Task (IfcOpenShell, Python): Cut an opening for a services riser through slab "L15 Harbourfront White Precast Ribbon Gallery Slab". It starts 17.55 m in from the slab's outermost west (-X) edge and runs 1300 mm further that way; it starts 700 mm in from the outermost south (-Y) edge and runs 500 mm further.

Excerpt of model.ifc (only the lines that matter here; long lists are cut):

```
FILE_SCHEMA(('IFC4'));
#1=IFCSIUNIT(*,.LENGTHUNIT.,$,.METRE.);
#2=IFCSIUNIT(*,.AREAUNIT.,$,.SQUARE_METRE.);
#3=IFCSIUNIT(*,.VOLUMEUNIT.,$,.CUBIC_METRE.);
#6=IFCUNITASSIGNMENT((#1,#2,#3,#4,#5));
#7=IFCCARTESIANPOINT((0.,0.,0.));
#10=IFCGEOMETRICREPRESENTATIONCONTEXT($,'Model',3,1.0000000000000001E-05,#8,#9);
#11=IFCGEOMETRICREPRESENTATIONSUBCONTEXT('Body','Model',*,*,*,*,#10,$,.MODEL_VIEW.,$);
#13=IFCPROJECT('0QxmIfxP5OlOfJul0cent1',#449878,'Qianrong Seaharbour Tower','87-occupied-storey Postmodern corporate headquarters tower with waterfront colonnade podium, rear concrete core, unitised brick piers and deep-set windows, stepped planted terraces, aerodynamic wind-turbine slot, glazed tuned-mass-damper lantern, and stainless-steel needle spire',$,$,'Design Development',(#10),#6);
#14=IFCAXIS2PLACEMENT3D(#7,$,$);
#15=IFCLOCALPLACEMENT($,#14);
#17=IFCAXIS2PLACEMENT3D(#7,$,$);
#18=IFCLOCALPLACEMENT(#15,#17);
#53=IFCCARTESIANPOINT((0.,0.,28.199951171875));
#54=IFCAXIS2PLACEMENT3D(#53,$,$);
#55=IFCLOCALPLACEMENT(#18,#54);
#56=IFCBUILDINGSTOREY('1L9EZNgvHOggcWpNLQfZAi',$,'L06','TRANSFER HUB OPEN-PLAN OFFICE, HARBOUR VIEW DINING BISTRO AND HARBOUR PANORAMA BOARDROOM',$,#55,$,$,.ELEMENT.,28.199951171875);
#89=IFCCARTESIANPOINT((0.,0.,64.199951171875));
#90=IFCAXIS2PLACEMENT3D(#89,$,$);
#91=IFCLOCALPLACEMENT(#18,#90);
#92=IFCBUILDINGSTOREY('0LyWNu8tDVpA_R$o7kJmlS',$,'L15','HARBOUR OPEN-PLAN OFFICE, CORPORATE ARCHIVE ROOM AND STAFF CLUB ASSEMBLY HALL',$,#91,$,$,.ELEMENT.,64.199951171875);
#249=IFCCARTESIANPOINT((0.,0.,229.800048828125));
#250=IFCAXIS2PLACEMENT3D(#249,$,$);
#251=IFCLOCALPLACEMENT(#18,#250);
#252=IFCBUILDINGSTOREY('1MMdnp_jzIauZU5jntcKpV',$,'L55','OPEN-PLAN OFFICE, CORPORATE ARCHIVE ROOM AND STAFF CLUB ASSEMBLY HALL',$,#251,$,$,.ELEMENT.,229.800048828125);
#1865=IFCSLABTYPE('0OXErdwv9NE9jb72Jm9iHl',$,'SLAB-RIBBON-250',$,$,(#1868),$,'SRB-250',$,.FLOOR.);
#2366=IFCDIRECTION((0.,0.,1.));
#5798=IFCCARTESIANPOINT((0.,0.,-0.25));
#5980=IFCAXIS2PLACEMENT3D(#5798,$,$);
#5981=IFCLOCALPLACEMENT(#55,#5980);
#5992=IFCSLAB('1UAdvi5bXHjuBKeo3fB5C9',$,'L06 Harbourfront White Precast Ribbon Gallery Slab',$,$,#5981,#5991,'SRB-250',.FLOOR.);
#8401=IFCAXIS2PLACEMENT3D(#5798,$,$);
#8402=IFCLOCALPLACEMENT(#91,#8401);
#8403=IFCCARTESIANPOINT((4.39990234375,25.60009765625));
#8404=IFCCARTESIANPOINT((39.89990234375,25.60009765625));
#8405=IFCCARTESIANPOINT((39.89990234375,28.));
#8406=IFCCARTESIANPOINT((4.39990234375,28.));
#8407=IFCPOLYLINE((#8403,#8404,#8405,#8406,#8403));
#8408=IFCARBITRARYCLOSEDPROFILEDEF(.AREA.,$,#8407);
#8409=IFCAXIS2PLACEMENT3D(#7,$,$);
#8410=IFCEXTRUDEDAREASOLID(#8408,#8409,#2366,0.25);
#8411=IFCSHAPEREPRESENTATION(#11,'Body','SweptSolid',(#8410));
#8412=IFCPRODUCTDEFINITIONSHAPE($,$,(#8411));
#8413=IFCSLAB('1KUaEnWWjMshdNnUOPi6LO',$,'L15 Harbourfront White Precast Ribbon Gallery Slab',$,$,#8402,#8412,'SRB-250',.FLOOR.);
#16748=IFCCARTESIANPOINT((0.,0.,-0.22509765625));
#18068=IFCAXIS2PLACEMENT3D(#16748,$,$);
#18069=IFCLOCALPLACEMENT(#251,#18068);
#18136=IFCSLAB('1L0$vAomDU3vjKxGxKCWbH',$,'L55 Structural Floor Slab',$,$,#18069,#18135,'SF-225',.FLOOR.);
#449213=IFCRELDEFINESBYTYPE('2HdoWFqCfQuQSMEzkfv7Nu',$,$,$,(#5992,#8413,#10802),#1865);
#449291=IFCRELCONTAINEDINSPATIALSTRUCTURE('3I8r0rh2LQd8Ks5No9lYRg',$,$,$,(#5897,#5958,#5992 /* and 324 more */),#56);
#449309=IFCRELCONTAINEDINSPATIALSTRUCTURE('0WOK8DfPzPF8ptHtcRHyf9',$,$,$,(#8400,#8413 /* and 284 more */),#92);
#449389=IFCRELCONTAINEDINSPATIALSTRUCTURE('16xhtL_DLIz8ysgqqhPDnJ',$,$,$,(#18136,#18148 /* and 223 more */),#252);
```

```python
import numpy as np
import ifcopenshell
import ifcopenshell.api.feature
import ifcopenshell.api.geometry
import ifcopenshell.api.root
import ifcopenshell.geom
import ifcopenshell.util.placement
import ifcopenshell.util.representation
import ifcopenshell.util.shape
import ifcopenshell.util.unit

model = ifcopenshell.open("model.ifc")
unit_scale = ifcopenshell.util.unit.calculate_unit_scale(model)
settings = ifcopenshell.geom.settings()


def volume(element):
    """Net volume in cubic metres, openings subtracted."""
    shape = ifcopenshell.geom.create_shape(settings, element)
    return ifcopenshell.util.shape.get_volume(shape.geometry)


slab = model.by_guid("1KUaEnWWjMshdNnUOPi6LO")
before = volume(slab)

# Extent in the slab's own axes, in metres. The edges named are its -X and -Y sides.
slab_shape = ifcopenshell.geom.create_shape(settings, slab)
vertices = ifcopenshell.util.shape.get_vertices(slab_shape.geometry)
x_min, y_min, bottom = vertices.min(axis=0)
top = vertices[:, 2].max()

opening = ifcopenshell.api.root.create_entity(model, ifc_class="IfcOpeningElement", name="Services riser opening", predefined_type="OPENING")
context = ifcopenshell.util.representation.get_context(model, "Model", "Body", "MODEL_VIEW")
width, depth = 1.3, 0.5
outline = [(0.0, 0.0), (width, 0.0), (width, depth), (0.0, depth), (0.0, 0.0)]
# Overshoot both faces by 50 mm so the cut is clean.
shape = ifcopenshell.api.geometry.add_slab_representation(
    model, context=context, depth=top - bottom + 0.1, polyline=outline
)
ifcopenshell.api.geometry.assign_representation(model, product=opening, representation=shape)

matrix = ifcopenshell.util.placement.get_local_placement(slab.ObjectPlacement)
matrix[:, 3] = matrix @ np.append(np.array([x_min + 17.55, y_min + 0.7, bottom - 0.05]) / unit_scale, 1.0)
ifcopenshell.api.geometry.edit_object_placement(model, product=opening, matrix=matrix, is_si=False)
ifcopenshell.api.feature.add_feature(model, feature=opening, element=slab)

after = volume(slab)

print(f"slab volume {before:.3f} -> {after:.3f} m3")

model.write("model_updated.ifc")
```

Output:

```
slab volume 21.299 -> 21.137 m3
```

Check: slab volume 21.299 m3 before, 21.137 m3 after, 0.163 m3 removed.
